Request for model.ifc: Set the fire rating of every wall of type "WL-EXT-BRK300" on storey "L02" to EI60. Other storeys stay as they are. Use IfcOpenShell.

First a look at what the model holds.

```python
import ifcopenshell
import ifcopenshell.util.element

model = ifcopenshell.open("model.ifc")
print(model.schema)
storey = next(s for s in model.by_type("IfcBuildingStorey") if s.Name == "L02")
walls = [e for e in ifcopenshell.util.element.get_decomposition(storey) if e.is_a("IfcWall")]
seen = {}
for e in walls:
    element_type = ifcopenshell.util.element.get_type(e)
    key = (element_type.Name if element_type != e and element_type else None, ifcopenshell.util.element.get_pset(e, "Pset_WallCommon", "FireRating"))
    seen[key] = seen.get(key, 0) + 1
for (name, value), count in sorted(seen.items(), key=str):
    print(count, "x", name, "|", value)
```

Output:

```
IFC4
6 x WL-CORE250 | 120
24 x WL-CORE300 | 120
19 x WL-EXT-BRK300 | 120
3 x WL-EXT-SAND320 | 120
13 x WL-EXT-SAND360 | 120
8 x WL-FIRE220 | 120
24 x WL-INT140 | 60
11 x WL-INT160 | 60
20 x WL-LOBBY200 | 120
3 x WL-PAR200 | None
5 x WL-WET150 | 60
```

```python
import ifcopenshell
import ifcopenshell.api.pset
import ifcopenshell.util.element

model = ifcopenshell.open("model.ifc")

storey = next(s for s in model.by_type("IfcBuildingStorey") if s.Name == "L02")
walls = [e for e in ifcopenshell.util.element.get_decomposition(storey) if e.is_a("IfcWall")]

count = 0
for e in walls:
    element_type = ifcopenshell.util.element.get_type(e)
    if element_type in (None, e) or element_type.Name != "WL-EXT-BRK300":
        continue
    # add_pset returns the element's existing set when there is one.
    pset = ifcopenshell.api.pset.add_pset(model, product=e, name="Pset_WallCommon")
    ifcopenshell.api.pset.edit_pset(model, pset=pset, properties={"FireRating": "EI60"})
    count += 1

print(count, "walls updated")

model.write("model_rev.ifc")
```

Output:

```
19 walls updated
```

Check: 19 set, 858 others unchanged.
